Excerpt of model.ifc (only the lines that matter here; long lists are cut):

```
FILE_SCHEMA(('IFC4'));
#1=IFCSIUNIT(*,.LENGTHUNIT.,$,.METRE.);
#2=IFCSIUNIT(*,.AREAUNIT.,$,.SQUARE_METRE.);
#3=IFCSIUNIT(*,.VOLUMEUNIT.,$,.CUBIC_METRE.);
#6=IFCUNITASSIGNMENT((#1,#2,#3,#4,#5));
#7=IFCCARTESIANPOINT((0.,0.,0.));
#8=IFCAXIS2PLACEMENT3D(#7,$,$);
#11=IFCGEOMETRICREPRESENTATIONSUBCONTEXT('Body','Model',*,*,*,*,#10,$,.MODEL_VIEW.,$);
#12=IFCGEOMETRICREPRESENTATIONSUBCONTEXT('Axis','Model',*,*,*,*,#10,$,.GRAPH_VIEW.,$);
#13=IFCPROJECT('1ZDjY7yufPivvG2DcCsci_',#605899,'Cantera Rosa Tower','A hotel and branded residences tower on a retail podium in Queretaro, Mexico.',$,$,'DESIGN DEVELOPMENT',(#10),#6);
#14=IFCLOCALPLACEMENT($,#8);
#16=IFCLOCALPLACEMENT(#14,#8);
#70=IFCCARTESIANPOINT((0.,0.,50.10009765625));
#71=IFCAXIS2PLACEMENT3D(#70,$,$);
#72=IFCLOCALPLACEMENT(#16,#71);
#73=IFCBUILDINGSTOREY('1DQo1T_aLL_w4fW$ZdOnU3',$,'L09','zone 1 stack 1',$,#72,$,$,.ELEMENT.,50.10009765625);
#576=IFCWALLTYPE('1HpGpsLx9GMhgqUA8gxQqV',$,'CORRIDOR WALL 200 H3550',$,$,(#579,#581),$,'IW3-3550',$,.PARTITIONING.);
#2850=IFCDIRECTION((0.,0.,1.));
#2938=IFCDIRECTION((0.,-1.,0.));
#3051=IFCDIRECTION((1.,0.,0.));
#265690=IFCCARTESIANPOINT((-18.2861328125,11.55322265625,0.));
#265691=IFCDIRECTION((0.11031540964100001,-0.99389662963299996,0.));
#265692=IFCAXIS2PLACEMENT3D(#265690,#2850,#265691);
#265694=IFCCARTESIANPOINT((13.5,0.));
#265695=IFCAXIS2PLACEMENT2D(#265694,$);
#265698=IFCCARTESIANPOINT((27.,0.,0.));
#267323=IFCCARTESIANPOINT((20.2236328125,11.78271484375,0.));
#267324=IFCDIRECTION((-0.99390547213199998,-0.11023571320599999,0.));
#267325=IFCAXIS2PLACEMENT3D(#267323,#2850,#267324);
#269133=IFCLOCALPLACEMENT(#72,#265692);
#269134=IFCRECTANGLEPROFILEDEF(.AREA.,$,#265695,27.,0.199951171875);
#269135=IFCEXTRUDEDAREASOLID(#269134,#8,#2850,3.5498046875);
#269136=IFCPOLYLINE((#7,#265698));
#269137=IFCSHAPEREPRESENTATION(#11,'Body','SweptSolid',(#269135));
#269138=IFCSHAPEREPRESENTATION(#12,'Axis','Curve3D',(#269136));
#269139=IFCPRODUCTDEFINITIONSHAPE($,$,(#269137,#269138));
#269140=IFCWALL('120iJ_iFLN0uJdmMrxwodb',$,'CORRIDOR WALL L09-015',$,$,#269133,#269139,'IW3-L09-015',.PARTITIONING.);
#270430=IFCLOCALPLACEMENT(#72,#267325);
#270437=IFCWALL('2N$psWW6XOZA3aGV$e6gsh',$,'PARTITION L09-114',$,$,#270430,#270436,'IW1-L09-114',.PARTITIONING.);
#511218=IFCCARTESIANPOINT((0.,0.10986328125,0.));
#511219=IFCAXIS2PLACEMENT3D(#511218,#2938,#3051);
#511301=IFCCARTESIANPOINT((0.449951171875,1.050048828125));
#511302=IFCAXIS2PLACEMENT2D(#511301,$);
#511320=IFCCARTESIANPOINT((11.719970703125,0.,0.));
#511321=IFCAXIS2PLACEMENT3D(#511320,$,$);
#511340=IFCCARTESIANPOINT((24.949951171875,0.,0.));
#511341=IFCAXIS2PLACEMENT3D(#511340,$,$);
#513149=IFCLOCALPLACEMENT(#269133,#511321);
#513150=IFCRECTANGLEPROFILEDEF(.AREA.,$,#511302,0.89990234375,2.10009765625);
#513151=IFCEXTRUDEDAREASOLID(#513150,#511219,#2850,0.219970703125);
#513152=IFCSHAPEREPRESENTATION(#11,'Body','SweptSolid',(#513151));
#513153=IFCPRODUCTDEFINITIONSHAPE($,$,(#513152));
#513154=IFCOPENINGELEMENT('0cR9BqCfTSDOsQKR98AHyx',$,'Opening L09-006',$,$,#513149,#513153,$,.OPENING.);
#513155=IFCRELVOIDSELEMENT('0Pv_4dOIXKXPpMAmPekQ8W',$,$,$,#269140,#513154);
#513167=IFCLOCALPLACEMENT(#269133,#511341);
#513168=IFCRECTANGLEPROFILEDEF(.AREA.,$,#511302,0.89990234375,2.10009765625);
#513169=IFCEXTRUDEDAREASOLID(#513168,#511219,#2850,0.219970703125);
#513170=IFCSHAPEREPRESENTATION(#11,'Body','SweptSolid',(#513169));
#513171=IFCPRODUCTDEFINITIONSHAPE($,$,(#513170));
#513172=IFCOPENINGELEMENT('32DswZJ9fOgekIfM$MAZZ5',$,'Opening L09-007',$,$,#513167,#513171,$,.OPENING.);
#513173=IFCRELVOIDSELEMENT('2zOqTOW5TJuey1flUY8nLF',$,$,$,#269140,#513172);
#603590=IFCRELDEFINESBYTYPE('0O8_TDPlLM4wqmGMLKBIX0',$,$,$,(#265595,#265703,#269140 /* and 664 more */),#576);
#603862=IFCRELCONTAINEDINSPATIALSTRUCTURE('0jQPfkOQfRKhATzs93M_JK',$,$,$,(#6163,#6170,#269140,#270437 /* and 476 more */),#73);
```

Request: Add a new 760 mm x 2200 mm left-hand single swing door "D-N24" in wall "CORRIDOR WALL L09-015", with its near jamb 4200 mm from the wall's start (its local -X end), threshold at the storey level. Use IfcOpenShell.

```python
import numpy as np
import ifcopenshell
import ifcopenshell.api.feature
import ifcopenshell.api.geometry
import ifcopenshell.api.root
import ifcopenshell.api.spatial
import ifcopenshell.geom
import ifcopenshell.util.element
import ifcopenshell.util.placement
import ifcopenshell.util.representation
import ifcopenshell.util.shape
import ifcopenshell.util.unit

model = ifcopenshell.open("model.ifc")
unit_scale = ifcopenshell.util.unit.calculate_unit_scale(model)
settings = ifcopenshell.geom.settings()


def volume(element):
    """Net volume in cubic metres, openings subtracted."""
    shape = ifcopenshell.geom.create_shape(settings, element)
    return ifcopenshell.util.shape.get_volume(shape.geometry)


wall = model.by_guid("120iJ_iFLN0uJdmMrxwodb")
storey = ifcopenshell.util.element.get_container(wall, ifc_class="IfcBuildingStorey")
context = ifcopenshell.util.representation.get_context(model, "Model", "Body", "MODEL_VIEW")
before = volume(wall)

width, height, from_end, sill = 0.76, 2.2, 4.2, 0.0  # metres

# The wall runs along its own X axis, and the end named is its -X end.
wall_shape = ifcopenshell.geom.create_shape(settings, wall)
x, y, z = ifcopenshell.util.shape.get_vertices(wall_shape.geometry).T
start = x.min() + from_end
face, thickness = float(y.min()), float(y.max() - y.min())
wall_matrix = ifcopenshell.util.placement.get_local_placement(wall.ObjectPlacement)
level = ifcopenshell.util.placement.get_local_placement(storey.ObjectPlacement)[2, 3]


def in_wall(x, y):
    """Placement at x, y metres in the wall's axes, at sill height."""
    matrix = wall_matrix.copy()
    matrix[:, 3] = wall_matrix @ np.array([x / unit_scale, y / unit_scale, 0.0, 1.0])
    matrix[2, 3] = level + sill / unit_scale
    return matrix


# Opening: a box that overshoots both wall faces by 50 mm.
opening = ifcopenshell.api.root.create_entity(model, ifc_class="IfcOpeningElement", predefined_type="OPENING")
box = ifcopenshell.api.geometry.add_wall_representation(
    model, context=context, length=width, height=height, thickness=thickness + 0.1
)
ifcopenshell.api.geometry.assign_representation(model, product=opening, representation=box)
ifcopenshell.api.geometry.edit_object_placement(model, product=opening, matrix=in_wall(start, face - 0.05), is_si=False)
ifcopenshell.api.feature.add_feature(model, feature=opening, element=wall)

door = ifcopenshell.api.root.create_entity(model, ifc_class="IfcDoor", name="D-N24", predefined_type="DOOR")
door.OverallWidth, door.OverallHeight = width / unit_scale, height / unit_scale
door.OperationType = "SINGLE_SWING_LEFT"
body = ifcopenshell.api.geometry.add_door_representation(
    model,
    context=context,
    overall_width=door.OverallWidth,
    overall_height=door.OverallHeight,
    operation_type="SINGLE_SWING_LEFT",
    lining_properties={"LiningDepth": thickness / unit_scale, "ThresholdDepth": thickness / unit_scale},
)
ifcopenshell.api.geometry.assign_representation(model, product=door, representation=body)
ifcopenshell.api.spatial.assign_container(model, products=[door], relating_structure=storey)
ifcopenshell.api.feature.add_filling(model, opening=opening, element=door)

# The lining spans the wall, so the door starts at the wall face.
ifcopenshell.api.geometry.edit_object_placement(model, product=door, matrix=in_wall(start, face), is_si=False)

after = volume(wall)

print(f"wall volume {before:.3f} -> {after:.3f} m3")

model.write("model_v2.ifc")
```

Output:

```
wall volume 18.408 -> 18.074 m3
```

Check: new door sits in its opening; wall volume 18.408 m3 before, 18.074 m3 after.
